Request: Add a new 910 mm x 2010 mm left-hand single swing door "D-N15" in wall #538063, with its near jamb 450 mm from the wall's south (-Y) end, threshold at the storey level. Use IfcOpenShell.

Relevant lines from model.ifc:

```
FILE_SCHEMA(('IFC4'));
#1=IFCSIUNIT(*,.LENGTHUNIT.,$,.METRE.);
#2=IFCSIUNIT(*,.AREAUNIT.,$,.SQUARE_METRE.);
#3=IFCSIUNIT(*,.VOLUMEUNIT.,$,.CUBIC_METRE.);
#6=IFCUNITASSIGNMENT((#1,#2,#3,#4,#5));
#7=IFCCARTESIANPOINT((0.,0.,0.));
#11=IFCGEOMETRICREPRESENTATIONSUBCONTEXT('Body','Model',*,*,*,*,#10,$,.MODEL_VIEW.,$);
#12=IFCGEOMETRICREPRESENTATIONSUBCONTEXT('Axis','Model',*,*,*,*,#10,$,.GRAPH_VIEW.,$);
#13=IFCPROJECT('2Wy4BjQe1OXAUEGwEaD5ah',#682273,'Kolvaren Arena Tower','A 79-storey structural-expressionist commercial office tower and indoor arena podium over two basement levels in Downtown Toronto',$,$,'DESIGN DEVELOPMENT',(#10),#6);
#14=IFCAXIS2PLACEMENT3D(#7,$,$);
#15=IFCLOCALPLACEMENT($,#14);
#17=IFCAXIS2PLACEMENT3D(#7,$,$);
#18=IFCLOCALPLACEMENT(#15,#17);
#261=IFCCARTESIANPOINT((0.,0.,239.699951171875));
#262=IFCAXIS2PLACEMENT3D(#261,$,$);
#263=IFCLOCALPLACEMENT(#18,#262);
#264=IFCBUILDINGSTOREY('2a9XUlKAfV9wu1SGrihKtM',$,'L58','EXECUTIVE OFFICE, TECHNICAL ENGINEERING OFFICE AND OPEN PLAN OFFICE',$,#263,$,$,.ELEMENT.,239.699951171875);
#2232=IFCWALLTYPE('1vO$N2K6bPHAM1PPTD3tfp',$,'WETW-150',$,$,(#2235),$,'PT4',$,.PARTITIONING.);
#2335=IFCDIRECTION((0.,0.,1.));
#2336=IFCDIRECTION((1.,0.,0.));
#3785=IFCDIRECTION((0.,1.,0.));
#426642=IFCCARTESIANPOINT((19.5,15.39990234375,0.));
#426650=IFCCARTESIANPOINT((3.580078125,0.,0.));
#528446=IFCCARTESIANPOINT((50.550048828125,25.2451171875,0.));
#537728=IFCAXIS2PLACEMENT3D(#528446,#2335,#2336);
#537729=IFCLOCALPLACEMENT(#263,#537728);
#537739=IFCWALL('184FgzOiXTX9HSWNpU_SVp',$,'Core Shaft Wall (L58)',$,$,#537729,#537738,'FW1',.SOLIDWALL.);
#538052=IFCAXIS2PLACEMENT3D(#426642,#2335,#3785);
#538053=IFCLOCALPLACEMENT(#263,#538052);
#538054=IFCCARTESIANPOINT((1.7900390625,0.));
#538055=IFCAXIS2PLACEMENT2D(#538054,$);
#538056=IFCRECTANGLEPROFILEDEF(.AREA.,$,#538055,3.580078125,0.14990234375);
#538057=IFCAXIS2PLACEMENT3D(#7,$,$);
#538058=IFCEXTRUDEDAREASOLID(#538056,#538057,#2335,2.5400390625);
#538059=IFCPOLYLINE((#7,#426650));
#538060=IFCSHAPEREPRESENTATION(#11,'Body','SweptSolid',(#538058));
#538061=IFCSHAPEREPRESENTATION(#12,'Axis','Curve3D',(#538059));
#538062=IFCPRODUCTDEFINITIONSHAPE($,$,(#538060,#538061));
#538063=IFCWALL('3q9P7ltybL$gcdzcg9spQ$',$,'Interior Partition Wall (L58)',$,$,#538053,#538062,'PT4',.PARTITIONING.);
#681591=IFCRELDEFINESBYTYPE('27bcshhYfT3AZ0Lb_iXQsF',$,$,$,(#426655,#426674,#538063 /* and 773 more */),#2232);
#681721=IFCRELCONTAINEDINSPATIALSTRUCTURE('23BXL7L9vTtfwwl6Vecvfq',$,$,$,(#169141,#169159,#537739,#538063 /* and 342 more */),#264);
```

```python
import numpy as np
import ifcopenshell
import ifcopenshell.api.feature
import ifcopenshell.api.geometry
import ifcopenshell.api.root
import ifcopenshell.api.spatial
import ifcopenshell.geom
import ifcopenshell.util.element
import ifcopenshell.util.placement
import ifcopenshell.util.representation
import ifcopenshell.util.shape
import ifcopenshell.util.unit

model = ifcopenshell.open("model.ifc")
unit_scale = ifcopenshell.util.unit.calculate_unit_scale(model)
settings = ifcopenshell.geom.settings()


def volume(element):
    """Net volume in cubic metres, openings subtracted."""
    shape = ifcopenshell.geom.create_shape(settings, element)
    return ifcopenshell.util.shape.get_volume(shape.geometry)


wall = model.by_id(538063)
storey = ifcopenshell.util.element.get_container(wall, ifc_class="IfcBuildingStorey")
context = ifcopenshell.util.representation.get_context(model, "Model", "Body", "MODEL_VIEW")
before = volume(wall)

width, height, from_end, sill = 0.91, 2.01, 0.45, 0.0  # metres

# The wall runs along its own X axis, and the end named is its -X end.
wall_shape = ifcopenshell.geom.create_shape(settings, wall)
x, y, z = ifcopenshell.util.shape.get_vertices(wall_shape.geometry).T
start = x.min() + from_end
face, thickness = float(y.min()), float(y.max() - y.min())
wall_matrix = ifcopenshell.util.placement.get_local_placement(wall.ObjectPlacement)
level = ifcopenshell.util.placement.get_local_placement(storey.ObjectPlacement)[2, 3]


def in_wall(x, y):
    """Placement at x, y metres in the wall's axes, at sill height."""
    matrix = wall_matrix.copy()
    matrix[:, 3] = wall_matrix @ np.array([x / unit_scale, y / unit_scale, 0.0, 1.0])
    matrix[2, 3] = level + sill / unit_scale
    return matrix


# Opening: a box that overshoots both wall faces by 50 mm.
opening = ifcopenshell.api.root.create_entity(model, ifc_class="IfcOpeningElement", predefined_type="OPENING")
box = ifcopenshell.api.geometry.add_wall_representation(
    model, context=context, length=width, height=height, thickness=thickness + 0.1
)
ifcopenshell.api.geometry.assign_representation(model, product=opening, representation=box)
ifcopenshell.api.geometry.edit_object_placement(model, product=opening, matrix=in_wall(start, face - 0.05), is_si=False)
ifcopenshell.api.feature.add_feature(model, feature=opening, element=wall)

door = ifcopenshell.api.root.create_entity(model, ifc_class="IfcDoor", name="D-N15", predefined_type="DOOR")
door.OverallWidth, door.OverallHeight = width / unit_scale, height / unit_scale
door.OperationType = "SINGLE_SWING_LEFT"
body = ifcopenshell.api.geometry.add_door_representation(
    model,
    context=context,
    overall_width=door.OverallWidth,
    overall_height=door.OverallHeight,
    operation_type="SINGLE_SWING_LEFT",
    lining_properties={"LiningDepth": thickness / unit_scale, "ThresholdDepth": thickness / unit_scale},
)
ifcopenshell.api.geometry.assign_representation(model, product=door, representation=body)
ifcopenshell.api.spatial.assign_container(model, products=[door], relating_structure=storey)
ifcopenshell.api.feature.add_filling(model, opening=opening, element=door)

# The lining spans the wall, so the door starts at the wall face.
ifcopenshell.api.geometry.edit_object_placement(model, product=door, matrix=in_wall(start, face), is_si=False)

after = volume(wall)

print(f"wall volume {before:.3f} -> {after:.3f} m3")

model.write("model_v2.ifc")
```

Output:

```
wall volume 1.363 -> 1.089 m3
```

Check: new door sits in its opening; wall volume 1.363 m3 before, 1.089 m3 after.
